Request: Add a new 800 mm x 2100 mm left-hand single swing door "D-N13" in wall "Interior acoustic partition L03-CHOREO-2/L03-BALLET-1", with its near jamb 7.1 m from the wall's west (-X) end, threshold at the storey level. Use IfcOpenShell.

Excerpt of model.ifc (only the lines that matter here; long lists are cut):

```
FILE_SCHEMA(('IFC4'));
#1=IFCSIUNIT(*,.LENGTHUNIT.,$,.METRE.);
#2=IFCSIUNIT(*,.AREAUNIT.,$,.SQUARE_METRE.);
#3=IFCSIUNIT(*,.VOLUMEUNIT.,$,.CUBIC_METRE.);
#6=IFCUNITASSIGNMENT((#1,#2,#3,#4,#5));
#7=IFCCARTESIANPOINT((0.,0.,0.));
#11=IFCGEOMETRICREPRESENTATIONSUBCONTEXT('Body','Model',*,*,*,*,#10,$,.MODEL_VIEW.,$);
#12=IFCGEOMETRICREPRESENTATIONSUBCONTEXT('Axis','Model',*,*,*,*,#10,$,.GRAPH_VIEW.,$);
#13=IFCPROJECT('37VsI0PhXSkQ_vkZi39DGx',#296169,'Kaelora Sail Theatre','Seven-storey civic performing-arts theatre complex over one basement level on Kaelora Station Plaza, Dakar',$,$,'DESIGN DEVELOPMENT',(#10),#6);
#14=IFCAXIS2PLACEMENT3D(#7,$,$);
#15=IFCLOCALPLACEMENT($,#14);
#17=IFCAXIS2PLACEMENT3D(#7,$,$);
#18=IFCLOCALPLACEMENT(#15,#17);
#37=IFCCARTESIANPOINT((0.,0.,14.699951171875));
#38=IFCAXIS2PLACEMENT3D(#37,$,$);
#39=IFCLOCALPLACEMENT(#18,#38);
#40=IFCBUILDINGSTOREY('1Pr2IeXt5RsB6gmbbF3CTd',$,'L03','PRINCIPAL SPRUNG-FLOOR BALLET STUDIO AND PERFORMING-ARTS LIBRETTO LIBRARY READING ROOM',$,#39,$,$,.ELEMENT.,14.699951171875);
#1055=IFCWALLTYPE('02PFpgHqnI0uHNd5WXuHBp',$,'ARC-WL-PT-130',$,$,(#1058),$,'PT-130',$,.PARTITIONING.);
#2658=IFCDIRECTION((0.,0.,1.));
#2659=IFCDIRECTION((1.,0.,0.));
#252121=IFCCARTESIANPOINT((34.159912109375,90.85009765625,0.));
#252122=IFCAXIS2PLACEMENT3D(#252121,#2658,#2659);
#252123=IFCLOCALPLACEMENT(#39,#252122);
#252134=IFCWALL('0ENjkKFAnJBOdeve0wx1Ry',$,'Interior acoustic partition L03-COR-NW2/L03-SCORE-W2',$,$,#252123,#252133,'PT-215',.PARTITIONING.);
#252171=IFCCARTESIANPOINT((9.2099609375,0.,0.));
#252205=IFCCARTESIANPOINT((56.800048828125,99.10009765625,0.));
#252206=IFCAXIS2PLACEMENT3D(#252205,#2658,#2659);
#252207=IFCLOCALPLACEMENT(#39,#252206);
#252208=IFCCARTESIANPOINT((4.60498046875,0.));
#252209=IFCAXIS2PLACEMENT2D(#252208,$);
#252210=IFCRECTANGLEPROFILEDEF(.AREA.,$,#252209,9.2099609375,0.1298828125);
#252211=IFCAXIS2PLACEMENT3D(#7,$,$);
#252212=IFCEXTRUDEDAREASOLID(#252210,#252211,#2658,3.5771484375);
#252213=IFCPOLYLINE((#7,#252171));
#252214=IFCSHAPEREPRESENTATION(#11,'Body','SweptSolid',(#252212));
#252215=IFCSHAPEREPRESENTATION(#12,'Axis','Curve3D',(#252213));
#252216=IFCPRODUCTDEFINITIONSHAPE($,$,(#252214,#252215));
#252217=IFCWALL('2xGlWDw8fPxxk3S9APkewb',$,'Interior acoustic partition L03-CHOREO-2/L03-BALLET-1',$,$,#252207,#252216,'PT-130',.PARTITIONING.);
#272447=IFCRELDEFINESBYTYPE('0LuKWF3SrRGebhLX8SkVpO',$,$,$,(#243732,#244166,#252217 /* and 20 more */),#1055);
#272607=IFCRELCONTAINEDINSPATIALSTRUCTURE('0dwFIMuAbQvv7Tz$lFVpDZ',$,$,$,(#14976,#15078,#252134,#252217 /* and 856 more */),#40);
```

```python
import numpy as np
import ifcopenshell
import ifcopenshell.api.feature
import ifcopenshell.api.geometry
import ifcopenshell.api.root
import ifcopenshell.api.spatial
import ifcopenshell.geom
import ifcopenshell.util.element
import ifcopenshell.util.placement
import ifcopenshell.util.representation
import ifcopenshell.util.shape
import ifcopenshell.util.unit

model = ifcopenshell.open("model.ifc")
unit_scale = ifcopenshell.util.unit.calculate_unit_scale(model)
settings = ifcopenshell.geom.settings()


def volume(element):
    """Net volume in cubic metres, openings subtracted."""
    shape = ifcopenshell.geom.create_shape(settings, element)
    return ifcopenshell.util.shape.get_volume(shape.geometry)


wall = model.by_guid("2xGlWDw8fPxxk3S9APkewb")
storey = ifcopenshell.util.element.get_container(wall, ifc_class="IfcBuildingStorey")
context = ifcopenshell.util.representation.get_context(model, "Model", "Body", "MODEL_VIEW")
before = volume(wall)

width, height, from_end, sill = 0.8, 2.1, 7.1, 0.0  # metres

# The wall runs along its own X axis, and the end named is its -X end.
wall_shape = ifcopenshell.geom.create_shape(settings, wall)
x, y, z = ifcopenshell.util.shape.get_vertices(wall_shape.geometry).T
start = x.min() + from_end
face, thickness = float(y.min()), float(y.max() - y.min())
wall_matrix = ifcopenshell.util.placement.get_local_placement(wall.ObjectPlacement)
level = ifcopenshell.util.placement.get_local_placement(storey.ObjectPlacement)[2, 3]


def in_wall(x, y):
    """Placement at x, y metres in the wall's axes, at sill height."""
    matrix = wall_matrix.copy()
    matrix[:, 3] = wall_matrix @ np.array([x / unit_scale, y / unit_scale, 0.0, 1.0])
    matrix[2, 3] = level + sill / unit_scale
    return matrix


# Opening: a box that overshoots both wall faces by 50 mm.
opening = ifcopenshell.api.root.create_entity(model, ifc_class="IfcOpeningElement", predefined_type="OPENING")
box = ifcopenshell.api.geometry.add_wall_representation(
    model, context=context, length=width, height=height, thickness=thickness + 0.1
)
ifcopenshell.api.geometry.assign_representation(model, product=opening, representation=box)
ifcopenshell.api.geometry.edit_object_placement(model, product=opening, matrix=in_wall(start, face - 0.05), is_si=False)
ifcopenshell.api.feature.add_feature(model, feature=opening, element=wall)

door = ifcopenshell.api.root.create_entity(model, ifc_class="IfcDoor", name="D-N13", predefined_type="DOOR")
door.OverallWidth, door.OverallHeight = width / unit_scale, height / unit_scale
door.OperationType = "SINGLE_SWING_LEFT"
body = ifcopenshell.api.geometry.add_door_representation(
    model,
    context=context,
    overall_width=door.OverallWidth,
    overall_height=door.OverallHeight,
    operation_type="SINGLE_SWING_LEFT",
    lining_properties={"LiningDepth": thickness / unit_scale, "ThresholdDepth": thickness / unit_scale},
)
ifcopenshell.api.geometry.assign_representation(model, product=door, representation=body)
ifcopenshell.api.spatial.assign_container(model, products=[door], relating_structure=storey)
ifcopenshell.api.feature.add_filling(model, opening=opening, element=door)

# The lining spans the wall, so the door starts at the wall face.
ifcopenshell.api.geometry.edit_object_placement(model, product=door, matrix=in_wall(start, face), is_si=False)

after = volume(wall)

print(f"wall volume {before:.3f} -> {after:.3f} m3")

model.write("model_v2.ifc")
```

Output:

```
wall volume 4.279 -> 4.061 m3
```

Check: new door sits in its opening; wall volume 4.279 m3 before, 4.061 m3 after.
